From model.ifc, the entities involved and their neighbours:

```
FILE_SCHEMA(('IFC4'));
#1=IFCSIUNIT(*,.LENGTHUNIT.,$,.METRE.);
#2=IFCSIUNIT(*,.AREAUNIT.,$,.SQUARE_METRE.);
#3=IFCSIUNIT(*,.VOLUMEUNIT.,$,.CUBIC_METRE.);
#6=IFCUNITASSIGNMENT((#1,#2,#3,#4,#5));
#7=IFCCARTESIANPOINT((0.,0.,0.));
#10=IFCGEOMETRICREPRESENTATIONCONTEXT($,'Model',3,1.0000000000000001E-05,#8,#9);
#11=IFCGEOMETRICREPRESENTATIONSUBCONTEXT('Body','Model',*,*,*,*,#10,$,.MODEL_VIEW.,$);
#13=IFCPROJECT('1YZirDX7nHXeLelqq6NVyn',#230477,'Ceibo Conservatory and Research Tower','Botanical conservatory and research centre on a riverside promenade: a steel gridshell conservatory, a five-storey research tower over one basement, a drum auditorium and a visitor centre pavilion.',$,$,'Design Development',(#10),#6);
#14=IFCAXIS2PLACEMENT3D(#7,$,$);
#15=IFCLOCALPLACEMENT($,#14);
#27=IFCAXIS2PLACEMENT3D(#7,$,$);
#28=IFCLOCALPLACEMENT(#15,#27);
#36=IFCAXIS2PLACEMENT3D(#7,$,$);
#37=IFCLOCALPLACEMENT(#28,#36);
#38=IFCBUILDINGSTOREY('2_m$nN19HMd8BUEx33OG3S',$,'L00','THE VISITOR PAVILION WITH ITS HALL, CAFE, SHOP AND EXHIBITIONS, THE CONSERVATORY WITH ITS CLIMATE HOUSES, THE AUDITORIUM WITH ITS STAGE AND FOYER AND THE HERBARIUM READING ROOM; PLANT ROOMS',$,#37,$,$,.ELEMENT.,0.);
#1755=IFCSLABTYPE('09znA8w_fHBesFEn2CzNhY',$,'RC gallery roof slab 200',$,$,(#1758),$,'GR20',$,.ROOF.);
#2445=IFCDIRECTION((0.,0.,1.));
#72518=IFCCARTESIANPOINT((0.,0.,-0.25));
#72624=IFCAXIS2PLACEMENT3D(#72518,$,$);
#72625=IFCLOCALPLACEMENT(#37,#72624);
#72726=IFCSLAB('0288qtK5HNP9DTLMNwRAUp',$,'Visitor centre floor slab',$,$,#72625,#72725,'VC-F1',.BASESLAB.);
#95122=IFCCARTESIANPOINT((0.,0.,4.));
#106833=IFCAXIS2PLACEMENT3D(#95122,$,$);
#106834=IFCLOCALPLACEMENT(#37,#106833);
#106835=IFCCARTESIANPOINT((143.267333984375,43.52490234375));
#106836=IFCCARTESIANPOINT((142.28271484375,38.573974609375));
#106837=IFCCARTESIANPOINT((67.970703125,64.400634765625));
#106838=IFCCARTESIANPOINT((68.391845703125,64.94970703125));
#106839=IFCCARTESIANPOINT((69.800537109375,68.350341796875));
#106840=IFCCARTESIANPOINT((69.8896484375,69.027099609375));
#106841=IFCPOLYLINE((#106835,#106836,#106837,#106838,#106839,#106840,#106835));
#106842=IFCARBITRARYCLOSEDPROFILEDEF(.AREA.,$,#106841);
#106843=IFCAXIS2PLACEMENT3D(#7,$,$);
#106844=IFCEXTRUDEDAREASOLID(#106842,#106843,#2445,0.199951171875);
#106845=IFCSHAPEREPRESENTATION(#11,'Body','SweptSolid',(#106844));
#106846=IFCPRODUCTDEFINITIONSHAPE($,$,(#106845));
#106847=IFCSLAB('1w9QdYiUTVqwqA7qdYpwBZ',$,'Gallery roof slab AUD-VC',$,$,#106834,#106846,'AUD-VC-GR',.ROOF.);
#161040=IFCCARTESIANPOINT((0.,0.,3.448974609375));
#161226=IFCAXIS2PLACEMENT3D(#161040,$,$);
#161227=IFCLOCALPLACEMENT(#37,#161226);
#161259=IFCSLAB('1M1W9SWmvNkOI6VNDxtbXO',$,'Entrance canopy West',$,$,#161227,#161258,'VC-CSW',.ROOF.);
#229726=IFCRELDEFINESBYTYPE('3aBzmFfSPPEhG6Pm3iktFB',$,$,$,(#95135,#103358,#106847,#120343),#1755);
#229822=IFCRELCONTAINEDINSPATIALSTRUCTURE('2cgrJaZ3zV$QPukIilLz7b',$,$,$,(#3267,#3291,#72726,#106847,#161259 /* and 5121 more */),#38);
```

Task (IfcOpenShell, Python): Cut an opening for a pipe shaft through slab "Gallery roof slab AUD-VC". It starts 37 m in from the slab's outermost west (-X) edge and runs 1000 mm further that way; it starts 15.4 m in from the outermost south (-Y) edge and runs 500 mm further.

```python
import numpy as np
import ifcopenshell
import ifcopenshell.api.feature
import ifcopenshell.api.geometry
import ifcopenshell.api.root
import ifcopenshell.geom
import ifcopenshell.util.placement
import ifcopenshell.util.representation
import ifcopenshell.util.shape
import ifcopenshell.util.unit

model = ifcopenshell.open("model.ifc")
unit_scale = ifcopenshell.util.unit.calculate_unit_scale(model)
settings = ifcopenshell.geom.settings()


def volume(element):
    """Net volume in cubic metres, openings subtracted."""
    shape = ifcopenshell.geom.create_shape(settings, element)
    return ifcopenshell.util.shape.get_volume(shape.geometry)


slab = model.by_id(106847)
before = volume(slab)

# Extent in the slab's own axes, in metres. The edges named are its -X and -Y sides.
slab_shape = ifcopenshell.geom.create_shape(settings, slab)
vertices = ifcopenshell.util.shape.get_vertices(slab_shape.geometry)
x_min, y_min, bottom = vertices.min(axis=0)
top = vertices[:, 2].max()

opening = ifcopenshell.api.root.create_entity(model, ifc_class="IfcOpeningElement", name="Pipe shaft opening", predefined_type="OPENING")
context = ifcopenshell.util.representation.get_context(model, "Model", "Body", "MODEL_VIEW")
width, depth = 1, 0.5
outline = [(0.0, 0.0), (width, 0.0), (width, depth), (0.0, depth), (0.0, 0.0)]
# Overshoot both faces by 50 mm so the cut is clean.
shape = ifcopenshell.api.geometry.add_slab_representation(
    model, context=context, depth=top - bottom + 0.1, polyline=outline
)
ifcopenshell.api.geometry.assign_representation(model, product=opening, representation=shape)

matrix = ifcopenshell.util.placement.get_local_placement(slab.ObjectPlacement)
matrix[:, 3] = matrix @ np.append(np.array([x_min + 37, y_min + 15.4, bottom - 0.05]) / unit_scale, 1.0)
ifcopenshell.api.geometry.edit_object_placement(model, product=opening, matrix=matrix, is_si=False)
ifcopenshell.api.feature.add_feature(model, feature=opening, element=slab)

after = volume(slab)

print(f"slab volume {before:.3f} -> {after:.3f} m3")

model.write("model_v2.ifc")
```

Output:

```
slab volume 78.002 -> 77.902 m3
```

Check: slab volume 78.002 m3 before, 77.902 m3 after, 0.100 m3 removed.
